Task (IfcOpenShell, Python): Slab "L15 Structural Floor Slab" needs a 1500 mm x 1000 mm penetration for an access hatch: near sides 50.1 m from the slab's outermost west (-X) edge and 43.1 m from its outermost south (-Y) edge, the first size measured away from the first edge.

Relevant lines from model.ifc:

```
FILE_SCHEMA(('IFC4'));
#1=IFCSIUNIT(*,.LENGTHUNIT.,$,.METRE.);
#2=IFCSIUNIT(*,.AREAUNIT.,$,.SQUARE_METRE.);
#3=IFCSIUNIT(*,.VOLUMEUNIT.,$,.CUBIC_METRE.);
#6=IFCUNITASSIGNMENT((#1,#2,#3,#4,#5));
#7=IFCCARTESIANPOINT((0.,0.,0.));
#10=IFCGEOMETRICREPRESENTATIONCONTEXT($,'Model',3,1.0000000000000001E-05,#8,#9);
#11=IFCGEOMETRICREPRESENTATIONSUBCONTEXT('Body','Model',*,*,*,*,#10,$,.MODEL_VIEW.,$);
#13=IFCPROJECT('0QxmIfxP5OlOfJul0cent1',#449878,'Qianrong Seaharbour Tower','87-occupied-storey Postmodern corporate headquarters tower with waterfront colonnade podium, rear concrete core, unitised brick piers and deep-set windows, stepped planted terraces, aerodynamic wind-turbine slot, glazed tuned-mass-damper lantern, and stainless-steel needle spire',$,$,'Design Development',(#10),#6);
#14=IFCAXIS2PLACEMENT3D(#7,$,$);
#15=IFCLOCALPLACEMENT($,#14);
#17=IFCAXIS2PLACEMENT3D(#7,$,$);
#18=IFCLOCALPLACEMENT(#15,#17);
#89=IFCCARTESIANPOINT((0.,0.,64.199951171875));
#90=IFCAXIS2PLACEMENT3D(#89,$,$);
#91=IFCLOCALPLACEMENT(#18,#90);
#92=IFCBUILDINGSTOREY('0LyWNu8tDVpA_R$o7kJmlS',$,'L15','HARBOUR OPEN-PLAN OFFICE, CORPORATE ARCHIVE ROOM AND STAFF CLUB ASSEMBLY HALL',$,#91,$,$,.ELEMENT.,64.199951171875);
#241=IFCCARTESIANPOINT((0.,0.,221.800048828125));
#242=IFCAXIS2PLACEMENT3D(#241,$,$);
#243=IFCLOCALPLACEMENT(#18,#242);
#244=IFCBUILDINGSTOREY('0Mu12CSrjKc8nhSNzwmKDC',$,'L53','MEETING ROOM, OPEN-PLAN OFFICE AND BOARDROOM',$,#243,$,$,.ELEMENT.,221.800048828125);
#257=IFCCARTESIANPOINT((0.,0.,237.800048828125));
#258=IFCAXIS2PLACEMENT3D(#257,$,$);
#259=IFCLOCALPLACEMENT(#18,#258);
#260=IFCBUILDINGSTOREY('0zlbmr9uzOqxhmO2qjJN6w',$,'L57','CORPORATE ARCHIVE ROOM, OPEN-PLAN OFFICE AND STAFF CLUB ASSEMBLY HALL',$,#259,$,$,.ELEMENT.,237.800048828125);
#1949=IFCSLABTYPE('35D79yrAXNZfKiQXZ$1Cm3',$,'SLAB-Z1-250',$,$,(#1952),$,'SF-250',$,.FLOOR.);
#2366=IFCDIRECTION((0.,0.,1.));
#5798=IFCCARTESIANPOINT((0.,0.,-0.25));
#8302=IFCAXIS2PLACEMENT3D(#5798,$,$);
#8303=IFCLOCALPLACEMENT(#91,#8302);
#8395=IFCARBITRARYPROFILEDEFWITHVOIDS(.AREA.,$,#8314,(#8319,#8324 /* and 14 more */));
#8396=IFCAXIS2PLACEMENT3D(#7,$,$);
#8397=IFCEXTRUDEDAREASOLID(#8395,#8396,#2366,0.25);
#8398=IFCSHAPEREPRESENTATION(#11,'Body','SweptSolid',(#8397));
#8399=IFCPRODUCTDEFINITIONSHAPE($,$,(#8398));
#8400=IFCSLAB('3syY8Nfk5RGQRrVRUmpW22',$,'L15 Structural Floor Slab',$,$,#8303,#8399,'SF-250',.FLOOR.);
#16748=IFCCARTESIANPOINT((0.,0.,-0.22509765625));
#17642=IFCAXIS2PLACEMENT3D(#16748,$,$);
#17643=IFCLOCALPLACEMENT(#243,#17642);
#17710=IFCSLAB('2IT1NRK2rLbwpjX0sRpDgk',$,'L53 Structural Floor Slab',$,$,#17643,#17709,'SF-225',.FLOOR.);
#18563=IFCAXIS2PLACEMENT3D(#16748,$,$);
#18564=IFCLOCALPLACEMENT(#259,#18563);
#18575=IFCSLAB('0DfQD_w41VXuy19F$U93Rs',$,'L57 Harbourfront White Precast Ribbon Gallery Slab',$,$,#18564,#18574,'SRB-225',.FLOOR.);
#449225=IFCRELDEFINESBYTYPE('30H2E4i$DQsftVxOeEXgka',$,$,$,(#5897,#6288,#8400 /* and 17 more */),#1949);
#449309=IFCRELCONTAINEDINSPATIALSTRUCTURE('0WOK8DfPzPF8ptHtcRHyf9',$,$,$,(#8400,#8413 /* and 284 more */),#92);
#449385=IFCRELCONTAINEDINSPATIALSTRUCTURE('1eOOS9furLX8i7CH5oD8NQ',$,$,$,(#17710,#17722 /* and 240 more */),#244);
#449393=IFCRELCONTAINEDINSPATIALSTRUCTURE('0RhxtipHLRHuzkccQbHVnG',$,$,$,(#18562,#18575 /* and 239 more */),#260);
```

```python
import numpy as np
import ifcopenshell
import ifcopenshell.api.feature
import ifcopenshell.api.geometry
import ifcopenshell.api.root
import ifcopenshell.geom
import ifcopenshell.util.placement
import ifcopenshell.util.representation
import ifcopenshell.util.shape
import ifcopenshell.util.unit

model = ifcopenshell.open("model.ifc")
unit_scale = ifcopenshell.util.unit.calculate_unit_scale(model)
settings = ifcopenshell.geom.settings()


def volume(element):
    """Net volume in cubic metres, openings subtracted."""
    shape = ifcopenshell.geom.create_shape(settings, element)
    return ifcopenshell.util.shape.get_volume(shape.geometry)


slab = model.by_guid("3syY8Nfk5RGQRrVRUmpW22")
before = volume(slab)

# Extent in the slab's own axes, in metres. The edges named are its -X and -Y sides.
slab_shape = ifcopenshell.geom.create_shape(settings, slab)
vertices = ifcopenshell.util.shape.get_vertices(slab_shape.geometry)
x_min, y_min, bottom = vertices.min(axis=0)
top = vertices[:, 2].max()

opening = ifcopenshell.api.root.create_entity(model, ifc_class="IfcOpeningElement", name="Access hatch opening", predefined_type="OPENING")
context = ifcopenshell.util.representation.get_context(model, "Model", "Body", "MODEL_VIEW")
width, depth = 1.5, 1
outline = [(0.0, 0.0), (width, 0.0), (width, depth), (0.0, depth), (0.0, 0.0)]
# Overshoot both faces by 50 mm so the cut is clean.
shape = ifcopenshell.api.geometry.add_slab_representation(
    model, context=context, depth=top - bottom + 0.1, polyline=outline
)
ifcopenshell.api.geometry.assign_representation(model, product=opening, representation=shape)

matrix = ifcopenshell.util.placement.get_local_placement(slab.ObjectPlacement)
matrix[:, 3] = matrix @ np.append(np.array([x_min + 50.1, y_min + 43.1, bottom - 0.05]) / unit_scale, 1.0)
ifcopenshell.api.geometry.edit_object_placement(model, product=opening, matrix=matrix, is_si=False)
ifcopenshell.api.feature.add_feature(model, feature=opening, element=slab)

after = volume(slab)

print(f"slab volume {before:.3f} -> {after:.3f} m3")

model.write("model_rev.ifc")
```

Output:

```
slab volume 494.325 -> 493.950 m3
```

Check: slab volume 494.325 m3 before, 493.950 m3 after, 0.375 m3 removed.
